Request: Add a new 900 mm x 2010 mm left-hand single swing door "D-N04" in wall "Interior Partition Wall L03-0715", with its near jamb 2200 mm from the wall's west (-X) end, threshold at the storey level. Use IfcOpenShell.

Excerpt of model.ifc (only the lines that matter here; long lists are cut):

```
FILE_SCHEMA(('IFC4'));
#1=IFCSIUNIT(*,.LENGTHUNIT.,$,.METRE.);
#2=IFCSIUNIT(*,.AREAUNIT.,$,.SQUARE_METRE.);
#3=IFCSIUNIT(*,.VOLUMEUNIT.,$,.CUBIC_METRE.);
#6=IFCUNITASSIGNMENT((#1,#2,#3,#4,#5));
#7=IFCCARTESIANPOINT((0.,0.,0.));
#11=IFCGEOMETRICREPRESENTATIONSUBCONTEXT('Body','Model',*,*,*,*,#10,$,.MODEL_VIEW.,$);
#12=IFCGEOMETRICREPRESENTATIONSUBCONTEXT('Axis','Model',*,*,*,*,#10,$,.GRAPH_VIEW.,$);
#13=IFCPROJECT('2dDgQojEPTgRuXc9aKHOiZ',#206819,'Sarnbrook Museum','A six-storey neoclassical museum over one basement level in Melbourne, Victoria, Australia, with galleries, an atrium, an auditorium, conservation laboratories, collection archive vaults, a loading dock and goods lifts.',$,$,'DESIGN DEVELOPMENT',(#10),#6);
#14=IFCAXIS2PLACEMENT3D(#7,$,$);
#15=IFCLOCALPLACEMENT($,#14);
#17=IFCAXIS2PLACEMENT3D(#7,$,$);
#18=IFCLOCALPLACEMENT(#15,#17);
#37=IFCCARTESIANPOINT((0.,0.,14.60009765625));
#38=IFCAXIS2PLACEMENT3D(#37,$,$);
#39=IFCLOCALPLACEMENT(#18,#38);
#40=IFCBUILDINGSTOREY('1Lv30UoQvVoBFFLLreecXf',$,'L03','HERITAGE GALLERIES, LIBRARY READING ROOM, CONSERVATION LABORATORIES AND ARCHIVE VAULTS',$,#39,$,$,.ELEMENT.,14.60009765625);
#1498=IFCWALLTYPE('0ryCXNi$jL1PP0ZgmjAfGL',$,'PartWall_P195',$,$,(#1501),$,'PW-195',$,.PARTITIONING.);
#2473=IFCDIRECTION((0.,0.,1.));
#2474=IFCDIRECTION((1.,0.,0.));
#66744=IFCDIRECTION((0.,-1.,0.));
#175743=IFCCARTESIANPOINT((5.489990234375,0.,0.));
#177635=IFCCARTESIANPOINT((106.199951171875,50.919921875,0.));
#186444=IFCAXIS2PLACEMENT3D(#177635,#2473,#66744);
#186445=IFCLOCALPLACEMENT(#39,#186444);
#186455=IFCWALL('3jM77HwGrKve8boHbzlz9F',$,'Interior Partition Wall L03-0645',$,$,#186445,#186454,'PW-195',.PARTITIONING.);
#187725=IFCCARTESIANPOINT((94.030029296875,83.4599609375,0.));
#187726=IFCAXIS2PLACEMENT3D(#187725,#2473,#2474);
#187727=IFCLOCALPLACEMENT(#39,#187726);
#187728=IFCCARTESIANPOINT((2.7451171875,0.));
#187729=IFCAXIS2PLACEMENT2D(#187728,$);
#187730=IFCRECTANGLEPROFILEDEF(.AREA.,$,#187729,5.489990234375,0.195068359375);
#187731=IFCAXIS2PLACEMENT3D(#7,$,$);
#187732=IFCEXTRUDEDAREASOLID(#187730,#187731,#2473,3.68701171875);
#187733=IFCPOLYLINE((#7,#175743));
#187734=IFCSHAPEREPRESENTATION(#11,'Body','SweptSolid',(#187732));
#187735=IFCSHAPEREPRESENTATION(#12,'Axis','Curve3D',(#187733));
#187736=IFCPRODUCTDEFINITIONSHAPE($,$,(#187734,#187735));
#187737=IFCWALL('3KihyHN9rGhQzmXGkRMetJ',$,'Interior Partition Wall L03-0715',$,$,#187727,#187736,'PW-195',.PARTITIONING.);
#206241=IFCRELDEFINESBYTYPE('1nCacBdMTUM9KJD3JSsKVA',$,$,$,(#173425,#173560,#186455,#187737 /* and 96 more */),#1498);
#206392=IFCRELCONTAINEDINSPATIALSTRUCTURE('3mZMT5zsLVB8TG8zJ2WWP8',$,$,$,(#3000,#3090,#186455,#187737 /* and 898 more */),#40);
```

```python
import numpy as np
import ifcopenshell
import ifcopenshell.api.feature
import ifcopenshell.api.geometry
import ifcopenshell.api.root
import ifcopenshell.api.spatial
import ifcopenshell.geom
import ifcopenshell.util.element
import ifcopenshell.util.placement
import ifcopenshell.util.representation
import ifcopenshell.util.shape
import ifcopenshell.util.unit

model = ifcopenshell.open("model.ifc")
unit_scale = ifcopenshell.util.unit.calculate_unit_scale(model)
settings = ifcopenshell.geom.settings()


def volume(element):
    """Net volume in cubic metres, openings subtracted."""
    shape = ifcopenshell.geom.create_shape(settings, element)
    return ifcopenshell.util.shape.get_volume(shape.geometry)


wall = model.by_id(187737)
storey = ifcopenshell.util.element.get_container(wall, ifc_class="IfcBuildingStorey")
context = ifcopenshell.util.representation.get_context(model, "Model", "Body", "MODEL_VIEW")
before = volume(wall)

width, height, from_end, sill = 0.9, 2.01, 2.2, 0.0  # metres

# The wall runs along its own X axis, and the end named is its -X end.
wall_shape = ifcopenshell.geom.create_shape(settings, wall)
x, y, z = ifcopenshell.util.shape.get_vertices(wall_shape.geometry).T
start = x.min() + from_end
face, thickness = float(y.min()), float(y.max() - y.min())
wall_matrix = ifcopenshell.util.placement.get_local_placement(wall.ObjectPlacement)
level = ifcopenshell.util.placement.get_local_placement(storey.ObjectPlacement)[2, 3]


def in_wall(x, y):
    """Placement at x, y metres in the wall's axes, at sill height."""
    matrix = wall_matrix.copy()
    matrix[:, 3] = wall_matrix @ np.array([x / unit_scale, y / unit_scale, 0.0, 1.0])
    matrix[2, 3] = level + sill / unit_scale
    return matrix


# Opening: a box that overshoots both wall faces by 50 mm.
opening = ifcopenshell.api.root.create_entity(model, ifc_class="IfcOpeningElement", predefined_type="OPENING")
box = ifcopenshell.api.geometry.add_wall_representation(
    model, context=context, length=width, height=height, thickness=thickness + 0.1
)
ifcopenshell.api.geometry.assign_representation(model, product=opening, representation=box)
ifcopenshell.api.geometry.edit_object_placement(model, product=opening, matrix=in_wall(start, face - 0.05), is_si=False)
ifcopenshell.api.feature.add_feature(model, feature=opening, element=wall)

door = ifcopenshell.api.root.create_entity(model, ifc_class="IfcDoor", name="D-N04", predefined_type="DOOR")
door.OverallWidth, door.OverallHeight = width / unit_scale, height / unit_scale
door.OperationType = "SINGLE_SWING_LEFT"
body = ifcopenshell.api.geometry.add_door_representation(
    model,
    context=context,
    overall_width=door.OverallWidth,
    overall_height=door.OverallHeight,
    operation_type="SINGLE_SWING_LEFT",
    lining_properties={"LiningDepth": thickness / unit_scale, "ThresholdDepth": thickness / unit_scale},
)
ifcopenshell.api.geometry.assign_representation(model, product=door, representation=body)
ifcopenshell.api.spatial.assign_container(model, products=[door], relating_structure=storey)
ifcopenshell.api.feature.add_filling(model, opening=opening, element=door)

# The lining spans the wall, so the door starts at the wall face.
ifcopenshell.api.geometry.edit_object_placement(model, product=door, matrix=in_wall(start, face), is_si=False)

after = volume(wall)

print(f"wall volume {before:.3f} -> {after:.3f} m3")

model.write("model_rev.ifc")
```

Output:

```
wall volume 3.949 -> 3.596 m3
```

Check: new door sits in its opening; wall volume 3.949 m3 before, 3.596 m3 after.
